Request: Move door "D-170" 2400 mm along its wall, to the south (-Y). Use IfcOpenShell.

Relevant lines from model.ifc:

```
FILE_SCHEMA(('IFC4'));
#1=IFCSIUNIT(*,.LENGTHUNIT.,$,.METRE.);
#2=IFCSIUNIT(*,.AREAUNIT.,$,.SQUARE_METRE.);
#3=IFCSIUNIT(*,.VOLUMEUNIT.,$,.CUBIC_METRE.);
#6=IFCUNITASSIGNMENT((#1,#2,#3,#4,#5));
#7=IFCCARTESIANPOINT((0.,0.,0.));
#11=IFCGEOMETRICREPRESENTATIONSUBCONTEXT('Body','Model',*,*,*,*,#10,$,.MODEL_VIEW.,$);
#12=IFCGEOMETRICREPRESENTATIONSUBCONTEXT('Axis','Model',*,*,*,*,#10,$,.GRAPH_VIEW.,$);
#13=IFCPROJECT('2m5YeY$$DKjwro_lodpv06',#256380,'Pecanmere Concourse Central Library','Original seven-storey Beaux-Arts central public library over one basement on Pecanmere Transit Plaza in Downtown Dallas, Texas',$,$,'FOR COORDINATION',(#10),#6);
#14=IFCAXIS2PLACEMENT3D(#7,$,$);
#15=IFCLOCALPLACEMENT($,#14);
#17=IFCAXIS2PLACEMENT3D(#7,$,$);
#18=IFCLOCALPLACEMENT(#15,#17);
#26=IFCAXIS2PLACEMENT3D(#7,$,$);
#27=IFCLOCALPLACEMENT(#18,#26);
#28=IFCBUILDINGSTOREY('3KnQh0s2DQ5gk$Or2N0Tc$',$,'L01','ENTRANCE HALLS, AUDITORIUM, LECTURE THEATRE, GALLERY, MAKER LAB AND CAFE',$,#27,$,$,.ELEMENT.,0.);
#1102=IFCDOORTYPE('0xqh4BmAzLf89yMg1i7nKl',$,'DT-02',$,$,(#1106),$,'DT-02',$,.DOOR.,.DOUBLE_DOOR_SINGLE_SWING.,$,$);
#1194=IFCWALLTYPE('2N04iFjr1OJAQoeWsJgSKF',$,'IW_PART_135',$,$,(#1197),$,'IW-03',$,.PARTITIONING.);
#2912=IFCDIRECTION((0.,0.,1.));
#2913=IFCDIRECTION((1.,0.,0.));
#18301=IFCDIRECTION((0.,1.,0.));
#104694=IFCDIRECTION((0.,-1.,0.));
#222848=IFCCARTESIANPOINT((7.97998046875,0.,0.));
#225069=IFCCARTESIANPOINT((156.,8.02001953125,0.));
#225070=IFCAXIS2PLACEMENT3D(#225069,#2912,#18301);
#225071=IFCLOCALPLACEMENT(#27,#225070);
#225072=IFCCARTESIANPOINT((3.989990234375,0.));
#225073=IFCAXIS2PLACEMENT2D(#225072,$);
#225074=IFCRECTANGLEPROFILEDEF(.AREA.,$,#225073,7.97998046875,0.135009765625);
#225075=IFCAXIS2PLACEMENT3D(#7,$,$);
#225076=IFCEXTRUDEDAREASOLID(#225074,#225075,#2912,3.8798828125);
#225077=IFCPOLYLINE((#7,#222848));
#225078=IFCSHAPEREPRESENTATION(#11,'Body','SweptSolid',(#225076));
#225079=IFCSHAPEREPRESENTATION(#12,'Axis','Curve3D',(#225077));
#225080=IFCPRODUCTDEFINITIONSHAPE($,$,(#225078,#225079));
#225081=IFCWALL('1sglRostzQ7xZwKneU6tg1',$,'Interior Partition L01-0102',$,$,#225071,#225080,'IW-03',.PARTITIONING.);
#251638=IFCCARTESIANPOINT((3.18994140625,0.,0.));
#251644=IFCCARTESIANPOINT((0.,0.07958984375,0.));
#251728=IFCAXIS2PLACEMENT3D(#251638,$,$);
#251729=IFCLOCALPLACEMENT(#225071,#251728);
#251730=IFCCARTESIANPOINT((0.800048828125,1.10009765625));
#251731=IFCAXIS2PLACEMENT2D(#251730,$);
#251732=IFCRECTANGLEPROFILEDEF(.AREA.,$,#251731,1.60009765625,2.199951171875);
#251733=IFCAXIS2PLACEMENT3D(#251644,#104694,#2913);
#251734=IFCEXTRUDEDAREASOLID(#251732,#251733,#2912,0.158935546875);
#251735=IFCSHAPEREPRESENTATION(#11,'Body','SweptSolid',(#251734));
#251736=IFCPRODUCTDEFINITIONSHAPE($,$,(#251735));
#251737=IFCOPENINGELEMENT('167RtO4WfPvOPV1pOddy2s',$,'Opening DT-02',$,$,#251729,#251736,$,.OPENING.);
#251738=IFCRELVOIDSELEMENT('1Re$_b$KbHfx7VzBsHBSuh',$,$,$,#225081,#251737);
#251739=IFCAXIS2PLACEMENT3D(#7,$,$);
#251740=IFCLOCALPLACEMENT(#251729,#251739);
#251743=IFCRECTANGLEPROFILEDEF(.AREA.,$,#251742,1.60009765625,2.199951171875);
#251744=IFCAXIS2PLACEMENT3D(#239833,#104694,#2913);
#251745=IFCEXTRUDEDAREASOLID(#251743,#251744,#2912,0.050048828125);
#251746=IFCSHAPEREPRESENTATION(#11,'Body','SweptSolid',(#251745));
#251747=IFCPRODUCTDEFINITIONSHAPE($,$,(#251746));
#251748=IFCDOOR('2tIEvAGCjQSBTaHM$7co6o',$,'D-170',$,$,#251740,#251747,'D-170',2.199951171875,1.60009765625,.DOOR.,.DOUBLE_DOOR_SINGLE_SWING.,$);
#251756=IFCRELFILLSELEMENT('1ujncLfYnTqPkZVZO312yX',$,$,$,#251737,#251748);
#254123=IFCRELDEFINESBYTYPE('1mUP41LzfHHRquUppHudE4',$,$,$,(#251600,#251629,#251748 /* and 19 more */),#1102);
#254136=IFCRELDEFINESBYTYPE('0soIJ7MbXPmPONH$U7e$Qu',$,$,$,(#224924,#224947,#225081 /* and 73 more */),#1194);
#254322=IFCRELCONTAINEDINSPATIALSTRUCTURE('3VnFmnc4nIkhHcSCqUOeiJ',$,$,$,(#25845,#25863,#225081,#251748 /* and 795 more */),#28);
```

```python
import ifcopenshell
import ifcopenshell.api.geometry
import ifcopenshell.util.placement

model = ifcopenshell.open("model.ifc")

door = model.by_id(251748)
opening = door.FillsVoids[0].RelatingOpeningElement
wall = opening.VoidsElements[0].RelatingBuildingElement

wall_matrix = ifcopenshell.util.placement.get_local_placement(wall.ObjectPlacement)
shift = wall_matrix[:3, 0] * -2.4
before = ifcopenshell.util.placement.get_local_placement(door.ObjectPlacement)[:3, 3].copy()

# The door is placed relative to its opening, so it follows when the opening moves.
matrix = ifcopenshell.util.placement.get_local_placement(opening.ObjectPlacement)
matrix[:3, 3] += shift
ifcopenshell.api.geometry.edit_object_placement(
    model, product=opening, matrix=matrix, is_si=False, should_transform_children=True
)

after = ifcopenshell.util.placement.get_local_placement(door.ObjectPlacement)[:3, 3]
print("door moved by", (after - before).round(3) + 0.0)

model.write("model_edited.ifc")
```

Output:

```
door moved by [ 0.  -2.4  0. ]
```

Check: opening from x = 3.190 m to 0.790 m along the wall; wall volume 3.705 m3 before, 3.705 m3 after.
